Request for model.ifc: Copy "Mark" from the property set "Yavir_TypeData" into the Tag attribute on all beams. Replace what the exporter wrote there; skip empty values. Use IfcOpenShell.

First a look at what the model holds.

```python
import ifcopenshell
import ifcopenshell.util.element

model = ifcopenshell.open("model.ifc")
print(model.schema)
beams = model.by_type("IfcBeam")
print(len(beams), "beams")
for e in beams[:8]:
    source = ifcopenshell.util.element.get_pset(e, "Yavir_TypeData", "Mark")
    target = e.Tag
    print(e.id(), repr(source), repr(target), sep=" | ")
```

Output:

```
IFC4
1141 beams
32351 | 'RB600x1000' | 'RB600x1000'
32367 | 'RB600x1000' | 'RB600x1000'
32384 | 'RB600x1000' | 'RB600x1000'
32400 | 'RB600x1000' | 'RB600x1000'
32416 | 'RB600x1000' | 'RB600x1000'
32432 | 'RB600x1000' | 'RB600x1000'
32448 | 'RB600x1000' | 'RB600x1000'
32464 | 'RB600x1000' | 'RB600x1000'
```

```python
import ifcopenshell
import ifcopenshell.util.element

model = ifcopenshell.open("model.ifc")

count = 0
for e in model.by_type("IfcBeam"):
    value = ifcopenshell.util.element.get_pset(e, "Yavir_TypeData", "Mark")
    current = e.Tag
    if not value or not value.strip() or current == value:
        continue
    e.Tag = value
    count += 1

print(count, "beams updated")

model.write("model_edited.ifc")
```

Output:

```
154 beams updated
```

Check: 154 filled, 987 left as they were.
